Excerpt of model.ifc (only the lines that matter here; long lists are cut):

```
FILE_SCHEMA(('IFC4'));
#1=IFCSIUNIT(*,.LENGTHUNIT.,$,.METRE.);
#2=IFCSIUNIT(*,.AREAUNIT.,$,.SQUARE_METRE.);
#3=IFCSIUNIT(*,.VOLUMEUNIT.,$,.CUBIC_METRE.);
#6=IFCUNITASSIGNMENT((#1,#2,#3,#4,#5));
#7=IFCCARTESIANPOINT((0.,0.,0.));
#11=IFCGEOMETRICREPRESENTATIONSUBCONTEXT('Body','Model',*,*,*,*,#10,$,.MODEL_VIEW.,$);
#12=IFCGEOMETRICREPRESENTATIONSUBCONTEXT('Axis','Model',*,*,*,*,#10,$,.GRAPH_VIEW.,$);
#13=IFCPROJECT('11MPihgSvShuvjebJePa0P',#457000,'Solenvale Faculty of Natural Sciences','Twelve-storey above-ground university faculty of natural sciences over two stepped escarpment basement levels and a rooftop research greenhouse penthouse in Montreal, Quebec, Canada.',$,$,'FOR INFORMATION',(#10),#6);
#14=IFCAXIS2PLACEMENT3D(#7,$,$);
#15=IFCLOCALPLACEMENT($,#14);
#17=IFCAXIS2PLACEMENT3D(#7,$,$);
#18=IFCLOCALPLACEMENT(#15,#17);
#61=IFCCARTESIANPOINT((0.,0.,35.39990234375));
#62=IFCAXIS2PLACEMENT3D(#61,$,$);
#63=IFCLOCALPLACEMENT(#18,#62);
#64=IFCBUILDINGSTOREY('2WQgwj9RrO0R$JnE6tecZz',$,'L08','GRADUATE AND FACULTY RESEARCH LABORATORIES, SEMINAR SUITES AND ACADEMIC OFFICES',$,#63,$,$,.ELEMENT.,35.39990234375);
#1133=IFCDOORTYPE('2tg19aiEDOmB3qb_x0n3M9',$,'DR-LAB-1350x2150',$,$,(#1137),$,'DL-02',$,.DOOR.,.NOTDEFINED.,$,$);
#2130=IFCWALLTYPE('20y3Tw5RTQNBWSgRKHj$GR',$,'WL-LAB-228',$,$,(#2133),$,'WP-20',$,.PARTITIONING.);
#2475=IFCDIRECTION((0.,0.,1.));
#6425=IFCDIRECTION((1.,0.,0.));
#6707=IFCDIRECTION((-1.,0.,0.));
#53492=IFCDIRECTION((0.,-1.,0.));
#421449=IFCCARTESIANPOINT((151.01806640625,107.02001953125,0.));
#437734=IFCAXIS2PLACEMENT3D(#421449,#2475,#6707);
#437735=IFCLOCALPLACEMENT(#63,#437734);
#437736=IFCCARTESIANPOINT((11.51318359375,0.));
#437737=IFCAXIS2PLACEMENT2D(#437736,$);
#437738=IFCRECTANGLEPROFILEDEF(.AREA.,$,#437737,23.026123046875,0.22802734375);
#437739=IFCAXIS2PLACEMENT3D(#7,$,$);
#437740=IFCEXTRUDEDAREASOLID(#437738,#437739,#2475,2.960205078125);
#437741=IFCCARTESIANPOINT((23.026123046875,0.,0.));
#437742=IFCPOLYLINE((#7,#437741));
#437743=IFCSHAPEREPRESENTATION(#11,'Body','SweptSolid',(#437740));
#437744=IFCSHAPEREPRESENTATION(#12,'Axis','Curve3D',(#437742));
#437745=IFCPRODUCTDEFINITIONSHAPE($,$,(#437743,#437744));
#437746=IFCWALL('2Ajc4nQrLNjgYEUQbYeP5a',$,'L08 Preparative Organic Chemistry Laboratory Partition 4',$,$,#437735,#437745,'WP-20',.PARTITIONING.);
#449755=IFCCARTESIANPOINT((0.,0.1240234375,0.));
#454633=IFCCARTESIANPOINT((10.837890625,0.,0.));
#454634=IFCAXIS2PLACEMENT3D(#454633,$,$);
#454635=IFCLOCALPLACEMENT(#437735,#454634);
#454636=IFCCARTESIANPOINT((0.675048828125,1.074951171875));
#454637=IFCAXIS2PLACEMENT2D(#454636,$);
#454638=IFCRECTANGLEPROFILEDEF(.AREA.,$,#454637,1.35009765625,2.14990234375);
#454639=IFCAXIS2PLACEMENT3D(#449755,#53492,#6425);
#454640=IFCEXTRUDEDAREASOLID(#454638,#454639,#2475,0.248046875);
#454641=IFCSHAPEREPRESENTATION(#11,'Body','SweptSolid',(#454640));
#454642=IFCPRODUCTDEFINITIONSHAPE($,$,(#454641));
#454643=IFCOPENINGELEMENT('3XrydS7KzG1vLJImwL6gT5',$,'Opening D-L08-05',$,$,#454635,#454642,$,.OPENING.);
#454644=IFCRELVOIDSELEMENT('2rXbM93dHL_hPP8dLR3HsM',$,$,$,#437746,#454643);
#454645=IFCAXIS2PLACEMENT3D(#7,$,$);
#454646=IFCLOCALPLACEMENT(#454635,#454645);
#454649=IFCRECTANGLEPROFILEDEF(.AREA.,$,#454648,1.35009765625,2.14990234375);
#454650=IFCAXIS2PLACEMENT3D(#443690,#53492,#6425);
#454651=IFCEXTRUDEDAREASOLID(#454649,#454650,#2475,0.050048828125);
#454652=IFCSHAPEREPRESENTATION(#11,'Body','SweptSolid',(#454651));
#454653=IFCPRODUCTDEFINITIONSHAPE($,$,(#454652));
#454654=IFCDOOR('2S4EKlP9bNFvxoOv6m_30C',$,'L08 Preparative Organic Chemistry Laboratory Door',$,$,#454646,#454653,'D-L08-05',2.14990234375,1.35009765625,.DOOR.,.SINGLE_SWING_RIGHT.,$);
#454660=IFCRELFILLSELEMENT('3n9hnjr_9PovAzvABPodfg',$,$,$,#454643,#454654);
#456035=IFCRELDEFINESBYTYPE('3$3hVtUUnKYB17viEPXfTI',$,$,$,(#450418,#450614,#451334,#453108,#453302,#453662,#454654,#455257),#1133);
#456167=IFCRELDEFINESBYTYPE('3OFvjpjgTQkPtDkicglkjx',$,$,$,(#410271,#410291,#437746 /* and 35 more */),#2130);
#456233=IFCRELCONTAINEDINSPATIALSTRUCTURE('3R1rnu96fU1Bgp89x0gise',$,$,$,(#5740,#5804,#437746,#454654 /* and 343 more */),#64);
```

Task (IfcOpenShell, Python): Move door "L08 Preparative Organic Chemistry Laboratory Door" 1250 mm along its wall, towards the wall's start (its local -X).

```python
import ifcopenshell
import ifcopenshell.api.geometry
import ifcopenshell.util.placement

model = ifcopenshell.open("model.ifc")

door = model.by_id(454654)
opening = door.FillsVoids[0].RelatingOpeningElement
wall = opening.VoidsElements[0].RelatingBuildingElement

wall_matrix = ifcopenshell.util.placement.get_local_placement(wall.ObjectPlacement)
shift = wall_matrix[:3, 0] * -1.25
before = ifcopenshell.util.placement.get_local_placement(door.ObjectPlacement)[:3, 3].copy()

# The door is placed relative to its opening, so it follows when the opening moves.
matrix = ifcopenshell.util.placement.get_local_placement(opening.ObjectPlacement)
matrix[:3, 3] += shift
ifcopenshell.api.geometry.edit_object_placement(
    model, product=opening, matrix=matrix, is_si=False, should_transform_children=True
)

after = ifcopenshell.util.placement.get_local_placement(door.ObjectPlacement)[:3, 3]
print("door moved by", (after - before).round(3) + 0.0)

model.write("model_v2.ifc")
```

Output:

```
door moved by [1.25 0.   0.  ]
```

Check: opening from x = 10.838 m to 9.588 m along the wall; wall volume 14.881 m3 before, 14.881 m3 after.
